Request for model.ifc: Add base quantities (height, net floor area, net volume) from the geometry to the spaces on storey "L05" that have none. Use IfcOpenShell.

First a look at what the model holds.

```python
import ifcopenshell
import ifcopenshell.util.element
import ifcopenshell.util.unit

model = ifcopenshell.open("model.ifc")
print(model.schema)
for unit_type in ("LENGTHUNIT", "AREAUNIT", "VOLUMEUNIT"):
    print(unit_type, ifcopenshell.util.unit.calculate_unit_scale(model, unit_type))
storey = next(s for s in model.by_type("IfcBuildingStorey") if s.Name == "L05")
spaces = [e for e in ifcopenshell.util.element.get_decomposition(storey) if e.is_a("IfcSpace")]
for e in sorted(spaces, key=lambda e: e.id()):
    print(e.id(), e.is_a(), e.Name, list(ifcopenshell.util.element.get_psets(e, qtos_only=True)), sep=" | ")
```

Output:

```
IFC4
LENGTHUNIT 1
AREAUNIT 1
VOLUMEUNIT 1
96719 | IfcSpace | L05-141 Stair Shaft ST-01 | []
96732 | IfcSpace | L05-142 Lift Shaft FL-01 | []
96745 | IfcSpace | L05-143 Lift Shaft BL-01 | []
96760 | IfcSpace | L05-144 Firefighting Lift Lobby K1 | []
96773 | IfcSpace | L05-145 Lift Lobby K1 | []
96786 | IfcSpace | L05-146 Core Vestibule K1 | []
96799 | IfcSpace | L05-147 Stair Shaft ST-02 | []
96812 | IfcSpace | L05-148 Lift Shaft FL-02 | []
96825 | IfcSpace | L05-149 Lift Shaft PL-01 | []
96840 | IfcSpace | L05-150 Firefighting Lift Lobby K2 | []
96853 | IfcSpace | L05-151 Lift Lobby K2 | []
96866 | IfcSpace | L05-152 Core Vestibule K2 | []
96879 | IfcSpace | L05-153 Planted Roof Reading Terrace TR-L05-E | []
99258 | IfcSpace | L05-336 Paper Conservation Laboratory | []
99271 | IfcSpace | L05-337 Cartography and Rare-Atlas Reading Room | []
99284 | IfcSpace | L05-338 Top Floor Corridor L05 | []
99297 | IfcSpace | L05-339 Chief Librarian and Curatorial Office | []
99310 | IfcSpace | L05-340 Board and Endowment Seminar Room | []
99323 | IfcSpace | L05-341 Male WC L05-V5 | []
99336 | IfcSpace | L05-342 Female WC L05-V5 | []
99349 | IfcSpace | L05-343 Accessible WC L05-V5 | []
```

```python
import ifcopenshell
import ifcopenshell.api.pset
import ifcopenshell.geom
import ifcopenshell.util.element
import ifcopenshell.util.shape
import ifcopenshell.util.unit

model = ifcopenshell.open("model.ifc")
unit_scale = ifcopenshell.util.unit.calculate_unit_scale(model)
area_scale = ifcopenshell.util.unit.calculate_unit_scale(model, "AREAUNIT")
volume_scale = ifcopenshell.util.unit.calculate_unit_scale(model, "VOLUMEUNIT")
settings = ifcopenshell.geom.settings()

storey = next(s for s in model.by_type("IfcBuildingStorey") if s.Name == "L05")
spaces = [e for e in ifcopenshell.util.element.get_decomposition(storey) if e.is_a("IfcSpace")]

for e in sorted(spaces, key=lambda e: e.id()):
    if ifcopenshell.util.element.get_psets(e, qtos_only=True, should_inherit=False):
        continue
    # Geometry comes back in metres, in the element's own axes.
    shape = ifcopenshell.geom.create_shape(settings, e)
    values = {
        "Height": ifcopenshell.util.shape.get_z(shape.geometry) / unit_scale,
        "NetFloorArea": ifcopenshell.util.shape.get_footprint_area(shape.geometry) / area_scale,
        "NetVolume": ifcopenshell.util.shape.get_volume(shape.geometry) / volume_scale,
    }
    qto = ifcopenshell.api.pset.add_qto(model, product=e, name="Qto_SpaceBaseQuantities")
    ifcopenshell.api.pset.edit_qto(model, qto=qto, properties=values)
    print(e.id(), {k: round(v, 3) for k, v in values.items()})

model.write("model_edited.ifc")
```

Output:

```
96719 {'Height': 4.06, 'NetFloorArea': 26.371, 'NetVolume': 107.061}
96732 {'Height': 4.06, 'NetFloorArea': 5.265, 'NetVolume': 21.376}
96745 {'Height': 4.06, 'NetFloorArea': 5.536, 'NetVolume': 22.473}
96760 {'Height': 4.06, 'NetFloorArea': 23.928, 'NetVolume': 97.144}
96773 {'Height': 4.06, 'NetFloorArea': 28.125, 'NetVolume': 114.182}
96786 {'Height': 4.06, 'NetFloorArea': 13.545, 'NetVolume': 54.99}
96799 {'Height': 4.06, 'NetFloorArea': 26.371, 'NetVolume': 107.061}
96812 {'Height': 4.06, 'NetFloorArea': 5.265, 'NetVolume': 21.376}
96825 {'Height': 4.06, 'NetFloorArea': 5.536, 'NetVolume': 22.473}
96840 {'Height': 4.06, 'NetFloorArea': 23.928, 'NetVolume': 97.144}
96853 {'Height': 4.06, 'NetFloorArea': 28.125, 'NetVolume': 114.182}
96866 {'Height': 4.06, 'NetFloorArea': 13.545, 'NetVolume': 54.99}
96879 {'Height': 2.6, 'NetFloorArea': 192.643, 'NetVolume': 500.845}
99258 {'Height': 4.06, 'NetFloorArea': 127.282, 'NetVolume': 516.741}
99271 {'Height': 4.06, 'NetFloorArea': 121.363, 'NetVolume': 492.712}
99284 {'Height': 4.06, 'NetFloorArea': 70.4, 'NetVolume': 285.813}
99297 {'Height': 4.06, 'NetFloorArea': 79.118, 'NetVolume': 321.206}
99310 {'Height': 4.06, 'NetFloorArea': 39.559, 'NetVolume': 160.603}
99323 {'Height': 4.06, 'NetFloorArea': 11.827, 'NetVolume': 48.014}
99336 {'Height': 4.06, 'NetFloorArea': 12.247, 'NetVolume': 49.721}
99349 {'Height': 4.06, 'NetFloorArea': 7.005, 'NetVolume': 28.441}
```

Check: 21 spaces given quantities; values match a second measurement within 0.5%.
